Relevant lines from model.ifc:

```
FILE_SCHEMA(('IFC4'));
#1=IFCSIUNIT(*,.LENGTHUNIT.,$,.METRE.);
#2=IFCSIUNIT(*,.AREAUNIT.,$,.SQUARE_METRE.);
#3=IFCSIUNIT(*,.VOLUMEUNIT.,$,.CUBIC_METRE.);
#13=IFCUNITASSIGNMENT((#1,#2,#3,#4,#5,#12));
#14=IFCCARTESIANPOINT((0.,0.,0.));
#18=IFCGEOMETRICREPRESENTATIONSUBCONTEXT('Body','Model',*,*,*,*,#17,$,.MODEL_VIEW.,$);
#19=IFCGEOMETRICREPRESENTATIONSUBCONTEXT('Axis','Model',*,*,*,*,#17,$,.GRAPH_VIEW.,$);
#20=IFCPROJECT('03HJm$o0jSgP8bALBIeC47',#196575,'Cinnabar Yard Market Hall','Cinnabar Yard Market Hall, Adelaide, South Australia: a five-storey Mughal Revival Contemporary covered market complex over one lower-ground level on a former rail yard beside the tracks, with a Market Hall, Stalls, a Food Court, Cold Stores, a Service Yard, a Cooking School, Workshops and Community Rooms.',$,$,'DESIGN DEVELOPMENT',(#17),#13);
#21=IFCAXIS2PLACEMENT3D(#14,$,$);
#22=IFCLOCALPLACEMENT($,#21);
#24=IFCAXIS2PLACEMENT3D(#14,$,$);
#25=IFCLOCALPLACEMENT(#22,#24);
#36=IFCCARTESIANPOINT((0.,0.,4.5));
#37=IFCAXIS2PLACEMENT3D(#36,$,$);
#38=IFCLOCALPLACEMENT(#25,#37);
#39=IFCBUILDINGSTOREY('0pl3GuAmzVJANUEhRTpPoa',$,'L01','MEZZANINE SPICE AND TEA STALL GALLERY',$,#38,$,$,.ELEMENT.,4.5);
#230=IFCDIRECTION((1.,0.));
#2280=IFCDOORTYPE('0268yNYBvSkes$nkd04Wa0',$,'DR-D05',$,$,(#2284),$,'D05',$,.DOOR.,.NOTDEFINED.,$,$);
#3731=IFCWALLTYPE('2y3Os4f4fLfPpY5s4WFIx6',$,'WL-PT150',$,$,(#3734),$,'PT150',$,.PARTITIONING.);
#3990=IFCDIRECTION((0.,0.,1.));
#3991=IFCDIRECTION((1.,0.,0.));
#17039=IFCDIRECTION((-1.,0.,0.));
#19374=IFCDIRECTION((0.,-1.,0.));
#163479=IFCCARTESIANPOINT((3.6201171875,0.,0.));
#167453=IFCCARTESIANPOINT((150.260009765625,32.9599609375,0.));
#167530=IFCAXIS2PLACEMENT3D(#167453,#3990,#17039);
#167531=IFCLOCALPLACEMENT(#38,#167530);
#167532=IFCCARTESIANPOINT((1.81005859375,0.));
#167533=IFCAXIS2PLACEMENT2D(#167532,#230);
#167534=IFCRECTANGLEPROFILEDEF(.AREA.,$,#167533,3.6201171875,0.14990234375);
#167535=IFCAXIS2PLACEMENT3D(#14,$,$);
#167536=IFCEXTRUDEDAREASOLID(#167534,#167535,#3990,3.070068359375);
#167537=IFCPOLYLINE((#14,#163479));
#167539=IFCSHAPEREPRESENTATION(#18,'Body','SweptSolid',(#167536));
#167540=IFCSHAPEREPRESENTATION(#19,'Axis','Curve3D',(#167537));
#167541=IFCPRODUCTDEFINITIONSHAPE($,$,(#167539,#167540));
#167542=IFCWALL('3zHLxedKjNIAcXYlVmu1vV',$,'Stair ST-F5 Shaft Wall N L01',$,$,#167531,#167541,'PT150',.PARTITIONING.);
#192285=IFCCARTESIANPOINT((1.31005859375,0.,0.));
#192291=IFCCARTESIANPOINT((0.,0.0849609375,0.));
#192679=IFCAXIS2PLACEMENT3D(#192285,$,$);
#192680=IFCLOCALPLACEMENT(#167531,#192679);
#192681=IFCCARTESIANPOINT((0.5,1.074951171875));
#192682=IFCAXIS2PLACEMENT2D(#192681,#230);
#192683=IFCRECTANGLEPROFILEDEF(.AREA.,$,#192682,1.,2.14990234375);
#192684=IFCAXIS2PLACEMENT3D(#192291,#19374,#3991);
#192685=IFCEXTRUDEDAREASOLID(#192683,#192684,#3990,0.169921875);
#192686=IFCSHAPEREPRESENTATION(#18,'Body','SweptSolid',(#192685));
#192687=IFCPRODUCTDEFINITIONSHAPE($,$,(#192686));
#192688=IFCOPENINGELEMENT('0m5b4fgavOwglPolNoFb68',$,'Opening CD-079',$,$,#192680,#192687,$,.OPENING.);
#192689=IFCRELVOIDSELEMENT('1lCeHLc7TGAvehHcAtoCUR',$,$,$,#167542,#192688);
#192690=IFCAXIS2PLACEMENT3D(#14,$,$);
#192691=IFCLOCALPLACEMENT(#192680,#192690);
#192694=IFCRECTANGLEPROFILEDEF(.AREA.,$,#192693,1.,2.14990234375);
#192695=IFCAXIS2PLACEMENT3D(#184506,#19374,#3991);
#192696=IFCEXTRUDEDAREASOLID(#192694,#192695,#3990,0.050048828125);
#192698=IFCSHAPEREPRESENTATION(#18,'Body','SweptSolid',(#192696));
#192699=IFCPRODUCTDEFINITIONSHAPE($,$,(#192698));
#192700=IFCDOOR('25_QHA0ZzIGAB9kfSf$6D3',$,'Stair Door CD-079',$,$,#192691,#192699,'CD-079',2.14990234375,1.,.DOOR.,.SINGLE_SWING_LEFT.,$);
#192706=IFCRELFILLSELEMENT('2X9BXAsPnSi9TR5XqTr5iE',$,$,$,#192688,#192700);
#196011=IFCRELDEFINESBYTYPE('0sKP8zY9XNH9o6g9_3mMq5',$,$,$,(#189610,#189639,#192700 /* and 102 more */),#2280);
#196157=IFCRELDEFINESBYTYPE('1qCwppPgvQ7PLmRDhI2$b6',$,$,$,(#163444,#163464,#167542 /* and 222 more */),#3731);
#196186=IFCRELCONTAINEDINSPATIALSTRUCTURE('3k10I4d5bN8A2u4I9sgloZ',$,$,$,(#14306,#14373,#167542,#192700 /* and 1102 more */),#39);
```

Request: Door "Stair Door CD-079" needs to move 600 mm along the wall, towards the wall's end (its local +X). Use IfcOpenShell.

```python
import ifcopenshell
import ifcopenshell.api.geometry
import ifcopenshell.util.placement

model = ifcopenshell.open("model.ifc")

door = model.by_guid("25_QHA0ZzIGAB9kfSf$6D3")
opening = door.FillsVoids[0].RelatingOpeningElement
wall = opening.VoidsElements[0].RelatingBuildingElement

wall_matrix = ifcopenshell.util.placement.get_local_placement(wall.ObjectPlacement)
shift = wall_matrix[:3, 0] * 0.6
before = ifcopenshell.util.placement.get_local_placement(door.ObjectPlacement)[:3, 3].copy()

# The door is placed relative to its opening, so it follows when the opening moves.
matrix = ifcopenshell.util.placement.get_local_placement(opening.ObjectPlacement)
matrix[:3, 3] += shift
ifcopenshell.api.geometry.edit_object_placement(
    model, product=opening, matrix=matrix, is_si=False, should_transform_children=True
)

after = ifcopenshell.util.placement.get_local_placement(door.ObjectPlacement)[:3, 3]
print("door moved by", (after - before).round(3) + 0.0)

model.write("model_v2.ifc")
```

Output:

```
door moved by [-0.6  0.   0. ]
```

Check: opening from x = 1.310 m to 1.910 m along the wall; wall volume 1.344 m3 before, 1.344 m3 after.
